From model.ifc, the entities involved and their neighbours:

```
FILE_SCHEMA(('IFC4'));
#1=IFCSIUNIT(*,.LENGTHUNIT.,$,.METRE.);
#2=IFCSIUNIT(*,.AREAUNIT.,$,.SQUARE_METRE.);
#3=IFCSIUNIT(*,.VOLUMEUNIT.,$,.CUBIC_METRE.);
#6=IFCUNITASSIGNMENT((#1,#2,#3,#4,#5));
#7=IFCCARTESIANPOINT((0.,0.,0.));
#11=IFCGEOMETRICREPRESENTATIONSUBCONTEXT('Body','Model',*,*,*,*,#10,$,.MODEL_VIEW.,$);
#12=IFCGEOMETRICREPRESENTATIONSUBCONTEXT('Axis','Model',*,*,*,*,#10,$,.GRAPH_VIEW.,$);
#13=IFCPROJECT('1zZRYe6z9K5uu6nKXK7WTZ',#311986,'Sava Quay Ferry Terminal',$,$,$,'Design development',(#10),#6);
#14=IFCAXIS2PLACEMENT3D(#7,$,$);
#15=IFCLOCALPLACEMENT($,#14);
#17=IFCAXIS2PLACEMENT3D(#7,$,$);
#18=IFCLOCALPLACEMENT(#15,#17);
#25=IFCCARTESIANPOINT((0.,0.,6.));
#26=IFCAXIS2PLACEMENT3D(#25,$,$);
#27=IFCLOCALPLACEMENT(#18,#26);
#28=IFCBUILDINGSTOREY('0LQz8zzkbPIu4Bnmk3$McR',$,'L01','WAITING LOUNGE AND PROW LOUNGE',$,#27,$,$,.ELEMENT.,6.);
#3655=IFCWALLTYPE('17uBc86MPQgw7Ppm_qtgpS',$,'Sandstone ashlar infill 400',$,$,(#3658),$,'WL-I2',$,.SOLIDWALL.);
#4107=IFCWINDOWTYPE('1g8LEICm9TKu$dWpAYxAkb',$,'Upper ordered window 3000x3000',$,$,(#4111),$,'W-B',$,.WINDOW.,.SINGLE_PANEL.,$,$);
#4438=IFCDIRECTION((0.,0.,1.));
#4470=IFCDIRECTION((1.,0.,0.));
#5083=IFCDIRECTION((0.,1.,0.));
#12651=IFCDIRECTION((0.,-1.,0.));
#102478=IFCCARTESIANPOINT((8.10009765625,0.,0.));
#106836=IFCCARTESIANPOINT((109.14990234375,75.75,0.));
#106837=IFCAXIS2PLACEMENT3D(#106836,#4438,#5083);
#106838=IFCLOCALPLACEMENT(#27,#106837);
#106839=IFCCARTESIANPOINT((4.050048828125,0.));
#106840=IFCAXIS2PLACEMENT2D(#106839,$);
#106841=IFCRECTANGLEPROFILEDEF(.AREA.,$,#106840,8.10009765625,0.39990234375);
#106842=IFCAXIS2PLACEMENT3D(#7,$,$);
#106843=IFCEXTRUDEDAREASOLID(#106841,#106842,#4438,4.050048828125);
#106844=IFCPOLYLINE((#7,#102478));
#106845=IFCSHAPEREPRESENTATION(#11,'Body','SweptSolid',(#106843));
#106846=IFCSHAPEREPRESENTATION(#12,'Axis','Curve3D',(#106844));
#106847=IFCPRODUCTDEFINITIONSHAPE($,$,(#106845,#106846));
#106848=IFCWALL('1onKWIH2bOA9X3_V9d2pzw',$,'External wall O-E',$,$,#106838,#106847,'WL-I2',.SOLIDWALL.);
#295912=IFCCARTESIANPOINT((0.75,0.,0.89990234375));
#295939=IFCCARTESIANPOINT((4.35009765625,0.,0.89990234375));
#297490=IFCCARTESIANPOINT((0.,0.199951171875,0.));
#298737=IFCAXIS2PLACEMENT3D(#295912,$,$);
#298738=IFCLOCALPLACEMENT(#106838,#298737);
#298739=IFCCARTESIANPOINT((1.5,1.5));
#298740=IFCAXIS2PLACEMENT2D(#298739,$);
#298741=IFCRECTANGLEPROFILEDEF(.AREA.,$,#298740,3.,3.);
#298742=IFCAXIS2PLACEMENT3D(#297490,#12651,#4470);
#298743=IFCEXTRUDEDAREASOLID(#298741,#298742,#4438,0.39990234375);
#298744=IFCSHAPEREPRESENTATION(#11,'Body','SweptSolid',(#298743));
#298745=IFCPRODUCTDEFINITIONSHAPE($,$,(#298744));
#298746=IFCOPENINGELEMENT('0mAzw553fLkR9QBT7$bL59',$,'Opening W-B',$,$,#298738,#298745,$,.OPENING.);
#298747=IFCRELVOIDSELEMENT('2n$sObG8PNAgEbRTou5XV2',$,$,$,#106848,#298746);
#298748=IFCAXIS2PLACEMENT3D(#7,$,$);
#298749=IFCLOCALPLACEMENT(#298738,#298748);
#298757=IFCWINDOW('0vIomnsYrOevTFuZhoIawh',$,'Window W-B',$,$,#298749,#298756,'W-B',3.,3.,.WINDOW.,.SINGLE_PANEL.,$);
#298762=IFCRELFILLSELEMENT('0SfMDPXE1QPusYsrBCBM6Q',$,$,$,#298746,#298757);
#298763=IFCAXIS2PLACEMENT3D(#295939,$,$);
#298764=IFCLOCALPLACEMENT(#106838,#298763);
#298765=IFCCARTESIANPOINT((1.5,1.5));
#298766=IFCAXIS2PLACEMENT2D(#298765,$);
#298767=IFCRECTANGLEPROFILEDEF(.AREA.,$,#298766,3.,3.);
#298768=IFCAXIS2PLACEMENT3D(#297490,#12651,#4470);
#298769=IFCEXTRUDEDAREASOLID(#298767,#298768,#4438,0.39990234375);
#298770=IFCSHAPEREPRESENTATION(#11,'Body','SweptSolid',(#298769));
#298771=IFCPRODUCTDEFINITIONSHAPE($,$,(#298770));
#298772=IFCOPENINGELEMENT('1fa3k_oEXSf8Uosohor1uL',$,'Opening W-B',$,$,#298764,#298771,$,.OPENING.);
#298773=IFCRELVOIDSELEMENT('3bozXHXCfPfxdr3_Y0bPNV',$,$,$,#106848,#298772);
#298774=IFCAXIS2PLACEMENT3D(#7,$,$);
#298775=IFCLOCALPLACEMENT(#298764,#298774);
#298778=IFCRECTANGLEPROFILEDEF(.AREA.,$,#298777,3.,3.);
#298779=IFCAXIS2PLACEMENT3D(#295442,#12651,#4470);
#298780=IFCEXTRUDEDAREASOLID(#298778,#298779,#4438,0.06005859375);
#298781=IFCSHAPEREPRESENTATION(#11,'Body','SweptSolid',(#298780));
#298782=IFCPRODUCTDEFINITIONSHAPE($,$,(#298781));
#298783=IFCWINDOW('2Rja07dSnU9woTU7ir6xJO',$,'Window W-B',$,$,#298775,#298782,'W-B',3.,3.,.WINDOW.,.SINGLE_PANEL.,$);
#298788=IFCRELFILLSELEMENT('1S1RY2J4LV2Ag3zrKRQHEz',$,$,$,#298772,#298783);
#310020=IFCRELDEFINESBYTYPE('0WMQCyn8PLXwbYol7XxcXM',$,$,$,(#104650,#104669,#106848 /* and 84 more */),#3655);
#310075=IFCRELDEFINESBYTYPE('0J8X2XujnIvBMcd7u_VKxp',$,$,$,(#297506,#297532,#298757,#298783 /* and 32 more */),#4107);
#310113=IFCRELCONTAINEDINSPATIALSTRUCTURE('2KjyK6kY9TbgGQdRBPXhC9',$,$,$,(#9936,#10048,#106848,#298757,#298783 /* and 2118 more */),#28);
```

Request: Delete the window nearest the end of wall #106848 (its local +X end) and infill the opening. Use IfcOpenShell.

```python
import ifcopenshell
import ifcopenshell.api.feature
import ifcopenshell.api.root
import ifcopenshell.geom
import ifcopenshell.util.shape

model = ifcopenshell.open("model.ifc")
settings = ifcopenshell.geom.settings()


def volume(element):
    """Net volume in cubic metres, openings subtracted."""
    shape = ifcopenshell.geom.create_shape(settings, element)
    return ifcopenshell.util.shape.get_volume(shape.geometry)


window = model.by_guid("2Rja07dSnU9woTU7ir6xJO")
opening = window.FillsVoids[0].RelatingOpeningElement
wall = opening.VoidsElements[0].RelatingBuildingElement
before = volume(wall)

ifcopenshell.api.root.remove_product(model, product=window)
ifcopenshell.api.feature.remove_feature(model, feature=opening)

after = volume(wall)

print(f"wall volume {before:.3f} -> {after:.3f} m3")

model.write("model_edited.ifc")
```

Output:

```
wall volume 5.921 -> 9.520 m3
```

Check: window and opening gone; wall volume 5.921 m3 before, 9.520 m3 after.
